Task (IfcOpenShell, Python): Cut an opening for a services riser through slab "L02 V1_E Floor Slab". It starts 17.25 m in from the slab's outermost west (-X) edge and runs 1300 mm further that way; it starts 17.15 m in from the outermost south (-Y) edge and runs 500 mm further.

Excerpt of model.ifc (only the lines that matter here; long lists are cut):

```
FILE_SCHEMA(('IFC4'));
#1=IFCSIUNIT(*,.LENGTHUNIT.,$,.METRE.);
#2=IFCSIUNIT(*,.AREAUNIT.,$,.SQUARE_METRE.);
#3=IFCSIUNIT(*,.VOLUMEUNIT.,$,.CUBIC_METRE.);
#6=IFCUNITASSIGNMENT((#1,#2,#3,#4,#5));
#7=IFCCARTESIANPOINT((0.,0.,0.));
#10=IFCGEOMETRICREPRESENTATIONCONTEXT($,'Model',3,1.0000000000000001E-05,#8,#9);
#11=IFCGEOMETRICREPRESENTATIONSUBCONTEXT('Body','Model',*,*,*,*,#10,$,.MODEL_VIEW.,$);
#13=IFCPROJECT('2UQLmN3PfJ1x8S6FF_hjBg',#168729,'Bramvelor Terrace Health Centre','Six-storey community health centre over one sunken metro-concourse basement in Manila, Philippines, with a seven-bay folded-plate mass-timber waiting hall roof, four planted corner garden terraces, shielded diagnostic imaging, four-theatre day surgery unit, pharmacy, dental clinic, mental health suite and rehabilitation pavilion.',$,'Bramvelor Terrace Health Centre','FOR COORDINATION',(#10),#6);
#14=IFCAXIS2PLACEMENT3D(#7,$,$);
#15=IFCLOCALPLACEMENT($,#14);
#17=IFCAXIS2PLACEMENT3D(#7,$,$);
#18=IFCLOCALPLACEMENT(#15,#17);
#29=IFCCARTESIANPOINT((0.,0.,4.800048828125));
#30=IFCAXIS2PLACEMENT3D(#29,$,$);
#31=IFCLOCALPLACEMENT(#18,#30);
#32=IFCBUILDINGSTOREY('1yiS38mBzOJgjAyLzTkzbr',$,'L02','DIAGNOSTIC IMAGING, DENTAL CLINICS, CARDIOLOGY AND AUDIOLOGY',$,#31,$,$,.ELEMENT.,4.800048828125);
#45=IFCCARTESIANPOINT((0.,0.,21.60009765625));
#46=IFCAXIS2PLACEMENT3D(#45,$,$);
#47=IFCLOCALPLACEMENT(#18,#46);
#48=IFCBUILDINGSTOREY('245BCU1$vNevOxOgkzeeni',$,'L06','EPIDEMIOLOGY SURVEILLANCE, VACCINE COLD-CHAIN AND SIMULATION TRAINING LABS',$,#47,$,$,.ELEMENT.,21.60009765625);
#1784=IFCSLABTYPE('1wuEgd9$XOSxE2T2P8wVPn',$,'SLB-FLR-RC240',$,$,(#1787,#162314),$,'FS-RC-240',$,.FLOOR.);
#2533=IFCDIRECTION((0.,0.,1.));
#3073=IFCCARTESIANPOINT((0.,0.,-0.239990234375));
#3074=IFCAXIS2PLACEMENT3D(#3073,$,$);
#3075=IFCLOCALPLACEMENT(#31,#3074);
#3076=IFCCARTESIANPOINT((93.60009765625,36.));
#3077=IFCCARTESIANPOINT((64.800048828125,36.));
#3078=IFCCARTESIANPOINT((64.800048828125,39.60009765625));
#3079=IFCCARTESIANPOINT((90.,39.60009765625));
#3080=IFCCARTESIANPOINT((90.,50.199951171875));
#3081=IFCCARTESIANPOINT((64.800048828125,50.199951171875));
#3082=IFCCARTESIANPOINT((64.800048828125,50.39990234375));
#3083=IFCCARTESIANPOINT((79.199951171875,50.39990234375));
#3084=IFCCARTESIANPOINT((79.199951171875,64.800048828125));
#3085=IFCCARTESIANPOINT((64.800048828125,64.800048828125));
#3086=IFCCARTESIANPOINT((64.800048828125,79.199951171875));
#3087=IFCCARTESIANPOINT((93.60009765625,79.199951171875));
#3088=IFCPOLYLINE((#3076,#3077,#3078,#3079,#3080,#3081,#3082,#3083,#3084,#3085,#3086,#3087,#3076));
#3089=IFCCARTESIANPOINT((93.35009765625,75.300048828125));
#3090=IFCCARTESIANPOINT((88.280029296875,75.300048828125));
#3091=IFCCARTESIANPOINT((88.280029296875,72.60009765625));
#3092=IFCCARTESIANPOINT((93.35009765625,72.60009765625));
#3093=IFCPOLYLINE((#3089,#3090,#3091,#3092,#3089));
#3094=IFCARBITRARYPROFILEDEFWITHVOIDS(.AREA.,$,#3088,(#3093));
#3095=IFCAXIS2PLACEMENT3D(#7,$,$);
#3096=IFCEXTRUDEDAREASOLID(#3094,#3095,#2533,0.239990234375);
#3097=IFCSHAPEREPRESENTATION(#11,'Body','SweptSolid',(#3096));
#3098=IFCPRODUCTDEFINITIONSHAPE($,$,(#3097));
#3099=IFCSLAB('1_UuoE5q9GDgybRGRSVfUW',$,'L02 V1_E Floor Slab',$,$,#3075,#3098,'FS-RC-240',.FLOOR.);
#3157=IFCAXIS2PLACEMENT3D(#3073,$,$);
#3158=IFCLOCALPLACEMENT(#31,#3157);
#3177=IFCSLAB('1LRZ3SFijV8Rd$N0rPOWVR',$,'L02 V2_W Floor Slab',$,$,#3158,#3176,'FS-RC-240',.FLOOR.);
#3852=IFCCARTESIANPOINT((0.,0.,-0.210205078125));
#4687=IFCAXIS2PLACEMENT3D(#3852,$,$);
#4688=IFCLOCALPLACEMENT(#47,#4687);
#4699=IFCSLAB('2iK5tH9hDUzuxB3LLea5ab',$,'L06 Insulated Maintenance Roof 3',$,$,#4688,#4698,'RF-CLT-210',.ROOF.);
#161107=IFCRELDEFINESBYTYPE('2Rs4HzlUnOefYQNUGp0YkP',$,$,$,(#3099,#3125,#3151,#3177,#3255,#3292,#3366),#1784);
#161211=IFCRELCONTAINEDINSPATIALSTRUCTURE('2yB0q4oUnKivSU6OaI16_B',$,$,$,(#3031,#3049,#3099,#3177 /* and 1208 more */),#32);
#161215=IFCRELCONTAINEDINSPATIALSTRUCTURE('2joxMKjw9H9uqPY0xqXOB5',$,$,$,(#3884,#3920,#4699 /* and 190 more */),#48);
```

```python
import numpy as np
import ifcopenshell
import ifcopenshell.api.feature
import ifcopenshell.api.geometry
import ifcopenshell.api.root
import ifcopenshell.geom
import ifcopenshell.util.placement
import ifcopenshell.util.representation
import ifcopenshell.util.shape
import ifcopenshell.util.unit

model = ifcopenshell.open("model.ifc")
unit_scale = ifcopenshell.util.unit.calculate_unit_scale(model)
settings = ifcopenshell.geom.settings()


def volume(element):
    """Net volume in cubic metres, openings subtracted."""
    shape = ifcopenshell.geom.create_shape(settings, element)
    return ifcopenshell.util.shape.get_volume(shape.geometry)


slab = model.by_id(3099)
before = volume(slab)

# Extent in the slab's own axes, in metres. The edges named are its -X and -Y sides.
slab_shape = ifcopenshell.geom.create_shape(settings, slab)
vertices = ifcopenshell.util.shape.get_vertices(slab_shape.geometry)
x_min, y_min, bottom = vertices.min(axis=0)
top = vertices[:, 2].max()

opening = ifcopenshell.api.root.create_entity(model, ifc_class="IfcOpeningElement", name="Services riser opening", predefined_type="OPENING")
context = ifcopenshell.util.representation.get_context(model, "Model", "Body", "MODEL_VIEW")
width, depth = 1.3, 0.5
outline = [(0.0, 0.0), (width, 0.0), (width, depth), (0.0, depth), (0.0, 0.0)]
# Overshoot both faces by 50 mm so the cut is clean.
shape = ifcopenshell.api.geometry.add_slab_representation(
    model, context=context, depth=top - bottom + 0.1, polyline=outline
)
ifcopenshell.api.geometry.assign_representation(model, product=opening, representation=shape)

matrix = ifcopenshell.util.placement.get_local_placement(slab.ObjectPlacement)
matrix[:, 3] = matrix @ np.append(np.array([x_min + 17.25, y_min + 17.15, bottom - 0.05]) / unit_scale, 1.0)
ifcopenshell.api.geometry.edit_object_placement(model, product=opening, matrix=matrix, is_si=False)
ifcopenshell.api.feature.add_feature(model, feature=opening, element=slab)

after = volume(slab)

print(f"slab volume {before:.3f} -> {after:.3f} m3")

model.write("model_edited.ifc")
```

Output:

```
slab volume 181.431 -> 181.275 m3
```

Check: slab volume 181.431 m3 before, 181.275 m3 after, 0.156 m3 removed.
